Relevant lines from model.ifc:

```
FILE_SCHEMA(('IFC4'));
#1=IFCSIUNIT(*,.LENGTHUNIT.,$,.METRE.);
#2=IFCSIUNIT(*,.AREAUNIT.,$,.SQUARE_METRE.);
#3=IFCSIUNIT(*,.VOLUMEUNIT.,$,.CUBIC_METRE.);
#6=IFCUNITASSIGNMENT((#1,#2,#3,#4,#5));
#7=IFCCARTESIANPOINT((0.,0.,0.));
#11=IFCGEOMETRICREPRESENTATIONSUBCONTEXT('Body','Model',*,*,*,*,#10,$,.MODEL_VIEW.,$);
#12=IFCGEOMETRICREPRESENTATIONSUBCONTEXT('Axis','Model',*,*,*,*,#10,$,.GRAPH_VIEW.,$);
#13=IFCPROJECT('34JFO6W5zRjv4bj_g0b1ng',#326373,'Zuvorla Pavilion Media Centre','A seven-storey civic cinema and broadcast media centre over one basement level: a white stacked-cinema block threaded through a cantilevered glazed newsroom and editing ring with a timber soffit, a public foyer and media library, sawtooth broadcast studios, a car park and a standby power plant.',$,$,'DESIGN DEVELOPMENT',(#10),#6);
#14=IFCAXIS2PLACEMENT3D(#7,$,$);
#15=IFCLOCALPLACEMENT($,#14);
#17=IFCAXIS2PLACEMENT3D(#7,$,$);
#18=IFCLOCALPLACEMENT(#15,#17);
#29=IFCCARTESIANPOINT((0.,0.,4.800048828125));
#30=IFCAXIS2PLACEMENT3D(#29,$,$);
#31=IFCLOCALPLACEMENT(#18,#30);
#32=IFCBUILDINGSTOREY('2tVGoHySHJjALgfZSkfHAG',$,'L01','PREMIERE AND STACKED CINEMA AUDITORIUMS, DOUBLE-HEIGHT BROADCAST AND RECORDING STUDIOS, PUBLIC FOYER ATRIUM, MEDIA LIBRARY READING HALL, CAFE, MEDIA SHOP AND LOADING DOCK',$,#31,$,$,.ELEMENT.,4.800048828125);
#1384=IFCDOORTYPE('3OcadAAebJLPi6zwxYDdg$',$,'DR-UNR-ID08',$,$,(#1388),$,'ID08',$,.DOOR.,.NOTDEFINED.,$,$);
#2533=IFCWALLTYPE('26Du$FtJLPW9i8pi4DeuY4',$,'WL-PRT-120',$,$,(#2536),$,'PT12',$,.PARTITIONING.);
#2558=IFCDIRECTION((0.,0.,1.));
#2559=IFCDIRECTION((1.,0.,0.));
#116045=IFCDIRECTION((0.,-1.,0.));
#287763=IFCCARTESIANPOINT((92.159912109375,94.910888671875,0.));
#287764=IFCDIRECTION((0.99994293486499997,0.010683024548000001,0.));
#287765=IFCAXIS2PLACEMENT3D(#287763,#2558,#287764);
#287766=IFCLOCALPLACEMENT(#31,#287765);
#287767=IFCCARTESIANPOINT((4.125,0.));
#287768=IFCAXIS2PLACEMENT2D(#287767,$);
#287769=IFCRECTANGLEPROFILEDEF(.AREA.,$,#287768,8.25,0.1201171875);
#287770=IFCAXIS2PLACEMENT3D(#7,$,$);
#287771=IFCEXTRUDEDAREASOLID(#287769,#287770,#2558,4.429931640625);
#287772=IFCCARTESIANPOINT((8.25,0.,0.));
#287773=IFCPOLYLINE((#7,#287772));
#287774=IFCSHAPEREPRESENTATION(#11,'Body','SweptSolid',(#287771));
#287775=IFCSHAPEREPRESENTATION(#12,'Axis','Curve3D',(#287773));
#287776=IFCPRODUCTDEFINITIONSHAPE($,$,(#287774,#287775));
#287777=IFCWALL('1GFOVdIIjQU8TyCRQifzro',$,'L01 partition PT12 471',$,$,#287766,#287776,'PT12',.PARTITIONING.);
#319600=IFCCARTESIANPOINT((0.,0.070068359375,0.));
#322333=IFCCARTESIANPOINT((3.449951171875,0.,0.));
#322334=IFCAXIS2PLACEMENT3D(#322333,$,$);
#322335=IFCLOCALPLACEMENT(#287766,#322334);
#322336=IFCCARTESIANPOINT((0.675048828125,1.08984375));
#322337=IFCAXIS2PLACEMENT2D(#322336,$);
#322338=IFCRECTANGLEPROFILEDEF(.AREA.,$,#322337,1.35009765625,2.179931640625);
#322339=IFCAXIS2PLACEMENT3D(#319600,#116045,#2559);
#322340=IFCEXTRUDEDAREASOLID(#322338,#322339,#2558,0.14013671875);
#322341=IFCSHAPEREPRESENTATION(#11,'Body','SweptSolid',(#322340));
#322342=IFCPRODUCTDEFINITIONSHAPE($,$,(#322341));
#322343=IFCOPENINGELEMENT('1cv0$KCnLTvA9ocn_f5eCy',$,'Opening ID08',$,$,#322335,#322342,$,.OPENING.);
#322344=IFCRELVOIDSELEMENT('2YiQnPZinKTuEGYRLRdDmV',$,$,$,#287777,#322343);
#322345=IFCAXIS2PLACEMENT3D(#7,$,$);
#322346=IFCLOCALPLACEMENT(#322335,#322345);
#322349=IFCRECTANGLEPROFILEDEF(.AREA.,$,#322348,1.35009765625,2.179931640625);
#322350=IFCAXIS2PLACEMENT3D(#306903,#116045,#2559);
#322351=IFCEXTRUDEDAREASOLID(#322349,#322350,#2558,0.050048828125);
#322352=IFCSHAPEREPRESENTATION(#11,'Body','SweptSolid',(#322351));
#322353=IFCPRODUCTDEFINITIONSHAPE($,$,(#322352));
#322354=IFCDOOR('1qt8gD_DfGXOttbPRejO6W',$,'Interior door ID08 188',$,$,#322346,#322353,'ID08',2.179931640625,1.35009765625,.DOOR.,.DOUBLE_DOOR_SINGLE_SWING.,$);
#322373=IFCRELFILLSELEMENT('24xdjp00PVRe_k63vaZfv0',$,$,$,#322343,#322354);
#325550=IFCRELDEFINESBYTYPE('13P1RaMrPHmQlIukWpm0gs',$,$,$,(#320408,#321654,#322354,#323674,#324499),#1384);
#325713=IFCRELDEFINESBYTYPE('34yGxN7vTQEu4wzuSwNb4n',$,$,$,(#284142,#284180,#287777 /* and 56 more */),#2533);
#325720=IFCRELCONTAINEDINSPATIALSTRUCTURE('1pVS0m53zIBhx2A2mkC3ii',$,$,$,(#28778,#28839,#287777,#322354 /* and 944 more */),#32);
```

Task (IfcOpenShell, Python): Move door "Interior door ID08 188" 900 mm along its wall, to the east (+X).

```python
import ifcopenshell
import ifcopenshell.api.geometry
import ifcopenshell.util.placement
import ifcopenshell.util.unit

model = ifcopenshell.open("model.ifc")
unit_scale = ifcopenshell.util.unit.calculate_unit_scale(model)

door = model.by_guid("1qt8gD_DfGXOttbPRejO6W")
opening = door.FillsVoids[0].RelatingOpeningElement
wall = opening.VoidsElements[0].RelatingBuildingElement

wall_matrix = ifcopenshell.util.placement.get_local_placement(wall.ObjectPlacement)
shift = wall_matrix[:3, 0] * 0.9 / unit_scale
before = ifcopenshell.util.placement.get_local_placement(door.ObjectPlacement)[:3, 3].copy()

# The door is placed relative to its opening, so it follows when the opening moves.
matrix = ifcopenshell.util.placement.get_local_placement(opening.ObjectPlacement)
matrix[:3, 3] += shift
ifcopenshell.api.geometry.edit_object_placement(
    model, product=opening, matrix=matrix, is_si=False, should_transform_children=True
)

after = ifcopenshell.util.placement.get_local_placement(door.ObjectPlacement)[:3, 3]
print("door moved by", (after - before).round(3) + 0.0)

model.write("model-out.ifc")
```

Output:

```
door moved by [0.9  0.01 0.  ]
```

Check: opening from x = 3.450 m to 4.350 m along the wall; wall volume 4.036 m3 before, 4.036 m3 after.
